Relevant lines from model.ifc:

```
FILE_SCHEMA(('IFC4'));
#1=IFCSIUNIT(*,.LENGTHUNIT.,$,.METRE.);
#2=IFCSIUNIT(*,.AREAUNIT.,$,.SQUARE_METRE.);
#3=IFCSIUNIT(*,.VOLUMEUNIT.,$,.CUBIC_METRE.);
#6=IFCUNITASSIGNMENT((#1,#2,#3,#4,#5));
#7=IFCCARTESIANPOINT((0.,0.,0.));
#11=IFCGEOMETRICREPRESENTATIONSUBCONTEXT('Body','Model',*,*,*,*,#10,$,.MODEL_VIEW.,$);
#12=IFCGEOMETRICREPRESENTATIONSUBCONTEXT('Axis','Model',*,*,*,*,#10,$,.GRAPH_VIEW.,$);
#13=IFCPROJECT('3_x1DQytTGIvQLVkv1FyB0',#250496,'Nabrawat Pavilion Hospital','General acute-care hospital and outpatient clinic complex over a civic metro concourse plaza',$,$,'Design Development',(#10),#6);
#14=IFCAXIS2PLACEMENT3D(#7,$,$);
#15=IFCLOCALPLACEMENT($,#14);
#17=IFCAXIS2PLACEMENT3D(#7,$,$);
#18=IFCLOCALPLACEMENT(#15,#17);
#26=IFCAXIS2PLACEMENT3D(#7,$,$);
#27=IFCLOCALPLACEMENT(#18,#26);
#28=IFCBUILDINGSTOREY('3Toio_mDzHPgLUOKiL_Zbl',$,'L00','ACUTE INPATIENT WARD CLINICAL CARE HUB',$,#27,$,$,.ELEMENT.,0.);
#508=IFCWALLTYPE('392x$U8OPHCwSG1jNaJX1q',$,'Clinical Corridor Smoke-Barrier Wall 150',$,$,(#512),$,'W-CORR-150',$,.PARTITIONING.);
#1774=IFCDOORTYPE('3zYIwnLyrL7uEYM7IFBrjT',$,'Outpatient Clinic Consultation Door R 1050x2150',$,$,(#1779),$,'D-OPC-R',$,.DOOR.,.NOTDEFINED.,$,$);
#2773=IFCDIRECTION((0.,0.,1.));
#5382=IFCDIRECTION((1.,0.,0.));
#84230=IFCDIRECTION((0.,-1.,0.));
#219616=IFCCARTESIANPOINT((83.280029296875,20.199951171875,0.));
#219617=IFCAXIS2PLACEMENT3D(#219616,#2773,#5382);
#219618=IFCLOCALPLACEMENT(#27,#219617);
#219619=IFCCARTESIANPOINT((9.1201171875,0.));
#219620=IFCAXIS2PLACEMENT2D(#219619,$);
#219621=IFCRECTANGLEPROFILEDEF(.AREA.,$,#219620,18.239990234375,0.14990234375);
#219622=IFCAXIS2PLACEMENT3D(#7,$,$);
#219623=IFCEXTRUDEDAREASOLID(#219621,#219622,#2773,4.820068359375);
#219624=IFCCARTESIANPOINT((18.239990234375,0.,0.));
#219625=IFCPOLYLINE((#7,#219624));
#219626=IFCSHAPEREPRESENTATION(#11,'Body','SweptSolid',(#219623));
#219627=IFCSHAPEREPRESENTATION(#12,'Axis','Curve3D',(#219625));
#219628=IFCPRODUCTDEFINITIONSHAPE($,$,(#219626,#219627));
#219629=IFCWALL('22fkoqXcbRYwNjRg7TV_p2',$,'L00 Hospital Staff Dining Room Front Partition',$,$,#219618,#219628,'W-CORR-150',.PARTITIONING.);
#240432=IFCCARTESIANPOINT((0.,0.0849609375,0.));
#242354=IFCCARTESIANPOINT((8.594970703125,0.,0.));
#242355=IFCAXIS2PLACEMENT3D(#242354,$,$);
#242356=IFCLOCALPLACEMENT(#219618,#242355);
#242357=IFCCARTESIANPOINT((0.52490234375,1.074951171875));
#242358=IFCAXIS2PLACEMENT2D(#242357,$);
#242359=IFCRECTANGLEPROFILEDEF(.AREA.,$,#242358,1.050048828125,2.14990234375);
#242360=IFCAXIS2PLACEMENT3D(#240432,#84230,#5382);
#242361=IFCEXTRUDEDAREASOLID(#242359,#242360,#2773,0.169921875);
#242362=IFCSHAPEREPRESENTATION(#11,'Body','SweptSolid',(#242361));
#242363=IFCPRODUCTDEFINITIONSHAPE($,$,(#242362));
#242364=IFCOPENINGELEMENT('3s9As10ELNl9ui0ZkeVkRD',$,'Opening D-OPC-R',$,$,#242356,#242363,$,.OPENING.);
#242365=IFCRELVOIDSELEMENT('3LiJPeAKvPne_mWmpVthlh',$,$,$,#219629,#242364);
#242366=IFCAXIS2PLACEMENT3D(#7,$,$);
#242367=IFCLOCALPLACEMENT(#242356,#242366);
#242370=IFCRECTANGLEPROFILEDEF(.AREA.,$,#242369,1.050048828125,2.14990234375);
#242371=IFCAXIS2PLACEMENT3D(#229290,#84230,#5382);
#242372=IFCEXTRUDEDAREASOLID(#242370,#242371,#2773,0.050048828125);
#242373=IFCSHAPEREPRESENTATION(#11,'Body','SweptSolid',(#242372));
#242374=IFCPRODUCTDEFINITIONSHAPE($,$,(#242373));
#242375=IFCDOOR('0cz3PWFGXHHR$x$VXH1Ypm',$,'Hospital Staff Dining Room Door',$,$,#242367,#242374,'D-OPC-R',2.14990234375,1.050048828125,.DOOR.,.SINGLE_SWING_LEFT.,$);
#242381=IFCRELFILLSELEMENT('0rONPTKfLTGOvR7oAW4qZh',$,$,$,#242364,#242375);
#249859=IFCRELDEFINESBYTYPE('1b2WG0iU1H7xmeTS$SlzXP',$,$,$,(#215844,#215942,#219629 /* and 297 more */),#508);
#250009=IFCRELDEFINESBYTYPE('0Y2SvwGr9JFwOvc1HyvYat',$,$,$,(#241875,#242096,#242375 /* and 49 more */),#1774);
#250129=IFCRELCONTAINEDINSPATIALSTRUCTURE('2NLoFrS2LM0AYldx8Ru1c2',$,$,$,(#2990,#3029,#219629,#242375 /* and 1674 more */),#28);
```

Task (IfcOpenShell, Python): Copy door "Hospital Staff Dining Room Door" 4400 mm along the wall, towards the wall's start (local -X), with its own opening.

```python
import ifcopenshell
import ifcopenshell.api.feature
import ifcopenshell.api.geometry
import ifcopenshell.api.root
import ifcopenshell.geom
import ifcopenshell.util.element
import ifcopenshell.util.placement
import ifcopenshell.util.shape

model = ifcopenshell.open("model.ifc")
settings = ifcopenshell.geom.settings()


def volume(element):
    """Net volume in cubic metres, openings subtracted."""
    shape = ifcopenshell.geom.create_shape(settings, element)
    return ifcopenshell.util.shape.get_volume(shape.geometry)


door = model.by_guid("0cz3PWFGXHHR$x$VXH1Ypm")
opening = door.FillsVoids[0].RelatingOpeningElement
wall = opening.VoidsElements[0].RelatingBuildingElement
before = volume(wall)
shift = ifcopenshell.util.placement.get_local_placement(wall.ObjectPlacement)[:3, 0] * -4.4

# copy_class copies the void relationship, type, container and properties, but no geometry.
new_opening = ifcopenshell.api.root.copy_class(model, product=opening)
new_opening.Representation = ifcopenshell.util.element.copy_deep(
    model, opening.Representation, exclude=["IfcGeometricRepresentationContext", "IfcRepresentationMap"]
)
new_door = ifcopenshell.api.root.copy_class(model, product=door)
new_door.Representation = ifcopenshell.util.element.copy_deep(
    model, door.Representation, exclude=["IfcGeometricRepresentationContext", "IfcRepresentationMap"]
)
new_door.Tag = None
ifcopenshell.api.feature.add_filling(model, opening=new_opening, element=new_door)

for old, new in ((opening, new_opening), (door, new_door)):
    matrix = ifcopenshell.util.placement.get_local_placement(old.ObjectPlacement)
    matrix[:3, 3] += shift
    ifcopenshell.api.geometry.edit_object_placement(model, product=new, matrix=matrix, is_si=False)

after = volume(wall)

print(f"wall volume {before:.3f} -> {after:.3f} m3")

model.write("model-out.ifc")
```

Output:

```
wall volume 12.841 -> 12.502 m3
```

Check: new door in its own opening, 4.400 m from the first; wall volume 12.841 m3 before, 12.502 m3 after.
